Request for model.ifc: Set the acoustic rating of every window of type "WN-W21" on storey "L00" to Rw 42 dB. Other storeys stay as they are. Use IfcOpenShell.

First a look at what the model holds.

```python
import ifcopenshell
import ifcopenshell.util.element

model = ifcopenshell.open("model.ifc")
print(model.schema)
storey = next(s for s in model.by_type("IfcBuildingStorey") if s.Name == "L00")
windows = [e for e in ifcopenshell.util.element.get_decomposition(storey) if e.is_a("IfcWindow")]
seen = {}
for e in windows:
    element_type = ifcopenshell.util.element.get_type(e)
    key = (element_type.Name if element_type != e and element_type else None, ifcopenshell.util.element.get_pset(e, "Pset_WindowCommon", "AcousticRating"))
    seen[key] = seen.get(key, 0) + 1
for (name, value), count in sorted(seen.items(), key=str):
    print(count, "x", name, "|", value)
```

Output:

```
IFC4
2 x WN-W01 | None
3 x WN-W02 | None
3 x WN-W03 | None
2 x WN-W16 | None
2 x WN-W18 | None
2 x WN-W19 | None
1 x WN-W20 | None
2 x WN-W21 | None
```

```python
import ifcopenshell
import ifcopenshell.api.pset
import ifcopenshell.util.element

model = ifcopenshell.open("model.ifc")

storey = next(s for s in model.by_type("IfcBuildingStorey") if s.Name == "L00")
windows = [e for e in ifcopenshell.util.element.get_decomposition(storey) if e.is_a("IfcWindow")]

count = 0
for e in windows:
    element_type = ifcopenshell.util.element.get_type(e)
    if element_type in (None, e) or element_type.Name != "WN-W21":
        continue
    # add_pset returns the element's existing set when there is one.
    pset = ifcopenshell.api.pset.add_pset(model, product=e, name="Pset_WindowCommon")
    ifcopenshell.api.pset.edit_pset(model, pset=pset, properties={"AcousticRating": "Rw 42 dB"})
    count += 1

print(count, "windows updated")

model.write("model-out.ifc")
```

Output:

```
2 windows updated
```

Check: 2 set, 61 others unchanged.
